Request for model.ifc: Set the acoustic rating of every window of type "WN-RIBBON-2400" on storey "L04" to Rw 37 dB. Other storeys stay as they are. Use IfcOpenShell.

First a look at what the model holds.

```python
import ifcopenshell
import ifcopenshell.util.element

model = ifcopenshell.open("model.ifc")
print(model.schema)
storey = next(s for s in model.by_type("IfcBuildingStorey") if s.Name == "L04")
windows = [e for e in ifcopenshell.util.element.get_decomposition(storey) if e.is_a("IfcWindow")]
seen = {}
for e in windows:
    element_type = ifcopenshell.util.element.get_type(e)
    key = (element_type.Name if element_type != e and element_type else None, ifcopenshell.util.element.get_pset(e, "Pset_WindowCommon", "AcousticRating"))
    seen[key] = seen.get(key, 0) + 1
for (name, value), count in sorted(seen.items(), key=str):
    print(count, "x", name, "|", value)
```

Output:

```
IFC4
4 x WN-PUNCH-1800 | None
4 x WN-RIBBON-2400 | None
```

```python
import ifcopenshell
import ifcopenshell.api.pset
import ifcopenshell.util.element

model = ifcopenshell.open("model.ifc")

storey = next(s for s in model.by_type("IfcBuildingStorey") if s.Name == "L04")
windows = [e for e in ifcopenshell.util.element.get_decomposition(storey) if e.is_a("IfcWindow")]

count = 0
for e in windows:
    element_type = ifcopenshell.util.element.get_type(e)
    if element_type in (None, e) or element_type.Name != "WN-RIBBON-2400":
        continue
    found = ifcopenshell.util.element.get_pset(e, "Pset_WindowCommon", should_inherit=False)
    if found:
        pset = model.by_id(found["id"])
        if len(ifcopenshell.util.element.get_elements_by_pset(pset)) > 1:
            pset = ifcopenshell.api.pset.unshare_pset(model, products=[e], pset=pset)[0]
    else:
        pset = ifcopenshell.api.pset.add_pset(model, product=e, name="Pset_WindowCommon")
    ifcopenshell.api.pset.edit_pset(model, pset=pset, properties={"AcousticRating": "Rw 37 dB"})
    count += 1

print(count, "windows updated")

model.write("model-out.ifc")
```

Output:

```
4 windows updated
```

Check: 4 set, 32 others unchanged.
